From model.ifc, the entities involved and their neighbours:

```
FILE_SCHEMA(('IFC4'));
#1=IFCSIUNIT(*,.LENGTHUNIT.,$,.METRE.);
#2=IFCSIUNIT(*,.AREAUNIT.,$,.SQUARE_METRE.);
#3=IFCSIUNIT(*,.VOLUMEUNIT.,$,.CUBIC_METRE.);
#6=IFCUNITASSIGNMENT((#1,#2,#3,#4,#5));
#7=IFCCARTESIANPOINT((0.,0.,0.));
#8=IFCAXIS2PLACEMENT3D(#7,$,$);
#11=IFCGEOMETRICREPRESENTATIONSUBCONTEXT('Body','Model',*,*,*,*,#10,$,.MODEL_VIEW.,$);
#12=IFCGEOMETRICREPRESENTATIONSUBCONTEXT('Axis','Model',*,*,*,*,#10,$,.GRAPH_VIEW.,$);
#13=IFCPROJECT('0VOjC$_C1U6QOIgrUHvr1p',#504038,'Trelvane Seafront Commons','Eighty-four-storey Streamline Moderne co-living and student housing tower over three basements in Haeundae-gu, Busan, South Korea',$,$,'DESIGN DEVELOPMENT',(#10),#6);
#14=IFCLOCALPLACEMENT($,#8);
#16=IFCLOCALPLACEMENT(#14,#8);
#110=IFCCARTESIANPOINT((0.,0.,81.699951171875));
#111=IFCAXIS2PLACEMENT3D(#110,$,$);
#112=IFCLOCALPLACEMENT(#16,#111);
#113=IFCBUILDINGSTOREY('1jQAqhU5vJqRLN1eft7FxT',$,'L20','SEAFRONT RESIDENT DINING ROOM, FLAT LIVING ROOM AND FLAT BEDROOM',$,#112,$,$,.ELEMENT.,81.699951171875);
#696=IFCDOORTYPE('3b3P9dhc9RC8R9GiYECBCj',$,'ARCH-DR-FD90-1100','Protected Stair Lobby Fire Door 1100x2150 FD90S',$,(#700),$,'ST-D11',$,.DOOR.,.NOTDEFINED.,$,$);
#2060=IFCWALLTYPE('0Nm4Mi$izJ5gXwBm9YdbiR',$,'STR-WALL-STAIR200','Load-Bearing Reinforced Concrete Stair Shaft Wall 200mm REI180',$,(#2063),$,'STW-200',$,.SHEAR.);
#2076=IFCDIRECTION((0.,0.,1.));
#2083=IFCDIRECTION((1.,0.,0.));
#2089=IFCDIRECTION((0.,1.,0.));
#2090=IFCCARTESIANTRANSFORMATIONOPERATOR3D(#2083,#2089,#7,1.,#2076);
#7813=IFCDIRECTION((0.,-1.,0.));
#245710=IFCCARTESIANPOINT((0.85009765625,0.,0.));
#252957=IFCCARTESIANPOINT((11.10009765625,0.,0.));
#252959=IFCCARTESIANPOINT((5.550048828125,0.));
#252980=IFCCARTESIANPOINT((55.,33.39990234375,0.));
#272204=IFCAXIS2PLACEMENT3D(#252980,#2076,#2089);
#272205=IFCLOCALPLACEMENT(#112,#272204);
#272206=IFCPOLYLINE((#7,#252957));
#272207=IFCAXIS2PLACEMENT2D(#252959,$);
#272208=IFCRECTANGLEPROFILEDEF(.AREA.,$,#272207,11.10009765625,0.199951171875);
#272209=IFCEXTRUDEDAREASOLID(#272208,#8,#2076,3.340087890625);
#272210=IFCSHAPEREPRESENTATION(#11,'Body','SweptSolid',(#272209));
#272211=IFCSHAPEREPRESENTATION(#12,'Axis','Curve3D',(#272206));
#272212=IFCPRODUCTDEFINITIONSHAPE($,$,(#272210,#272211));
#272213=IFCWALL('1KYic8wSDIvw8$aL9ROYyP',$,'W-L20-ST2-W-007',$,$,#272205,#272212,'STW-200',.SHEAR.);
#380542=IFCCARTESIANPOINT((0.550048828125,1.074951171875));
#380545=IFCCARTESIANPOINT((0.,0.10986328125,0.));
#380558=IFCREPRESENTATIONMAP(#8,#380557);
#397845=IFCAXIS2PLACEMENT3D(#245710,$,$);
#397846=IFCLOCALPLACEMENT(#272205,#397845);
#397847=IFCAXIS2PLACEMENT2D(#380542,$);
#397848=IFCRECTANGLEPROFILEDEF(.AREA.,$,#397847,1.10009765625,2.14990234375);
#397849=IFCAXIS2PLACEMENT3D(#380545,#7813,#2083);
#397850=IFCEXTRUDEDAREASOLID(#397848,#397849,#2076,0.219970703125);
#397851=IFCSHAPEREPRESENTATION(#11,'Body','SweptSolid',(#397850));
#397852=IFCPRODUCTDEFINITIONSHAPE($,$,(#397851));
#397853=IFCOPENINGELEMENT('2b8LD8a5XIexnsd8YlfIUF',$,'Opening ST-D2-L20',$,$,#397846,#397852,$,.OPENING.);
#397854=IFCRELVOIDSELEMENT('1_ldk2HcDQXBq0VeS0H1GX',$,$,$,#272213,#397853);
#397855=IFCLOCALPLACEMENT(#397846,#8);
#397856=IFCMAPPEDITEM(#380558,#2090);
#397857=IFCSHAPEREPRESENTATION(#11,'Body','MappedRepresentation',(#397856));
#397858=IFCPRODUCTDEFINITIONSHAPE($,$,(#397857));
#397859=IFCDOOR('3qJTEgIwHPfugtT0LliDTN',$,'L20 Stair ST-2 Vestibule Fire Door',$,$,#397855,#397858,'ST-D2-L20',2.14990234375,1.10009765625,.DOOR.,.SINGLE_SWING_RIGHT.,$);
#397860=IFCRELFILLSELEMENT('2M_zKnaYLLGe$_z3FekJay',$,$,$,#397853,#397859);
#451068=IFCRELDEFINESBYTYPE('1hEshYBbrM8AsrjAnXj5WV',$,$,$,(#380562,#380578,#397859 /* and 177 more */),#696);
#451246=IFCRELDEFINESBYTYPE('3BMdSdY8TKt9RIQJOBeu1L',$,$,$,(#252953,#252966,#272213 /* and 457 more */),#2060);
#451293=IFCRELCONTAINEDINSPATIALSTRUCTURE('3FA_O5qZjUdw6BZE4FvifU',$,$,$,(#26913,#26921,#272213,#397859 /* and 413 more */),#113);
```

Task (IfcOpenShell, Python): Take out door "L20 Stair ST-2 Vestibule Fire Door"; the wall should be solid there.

```python
import ifcopenshell
import ifcopenshell.api.feature
import ifcopenshell.api.root
import ifcopenshell.geom
import ifcopenshell.util.shape

model = ifcopenshell.open("model.ifc")
settings = ifcopenshell.geom.settings()


def volume(element):
    """Net volume in cubic metres, openings subtracted."""
    shape = ifcopenshell.geom.create_shape(settings, element)
    return ifcopenshell.util.shape.get_volume(shape.geometry)


door = model.by_guid("3qJTEgIwHPfugtT0LliDTN")
opening = door.FillsVoids[0].RelatingOpeningElement
wall = opening.VoidsElements[0].RelatingBuildingElement
before = volume(wall)

ifcopenshell.api.root.remove_product(model, product=door)
ifcopenshell.api.feature.remove_feature(model, feature=opening)

after = volume(wall)

print(f"wall volume {before:.3f} -> {after:.3f} m3")

model.write("model_edited.ifc")
```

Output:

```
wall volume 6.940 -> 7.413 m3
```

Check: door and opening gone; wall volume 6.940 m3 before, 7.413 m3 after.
